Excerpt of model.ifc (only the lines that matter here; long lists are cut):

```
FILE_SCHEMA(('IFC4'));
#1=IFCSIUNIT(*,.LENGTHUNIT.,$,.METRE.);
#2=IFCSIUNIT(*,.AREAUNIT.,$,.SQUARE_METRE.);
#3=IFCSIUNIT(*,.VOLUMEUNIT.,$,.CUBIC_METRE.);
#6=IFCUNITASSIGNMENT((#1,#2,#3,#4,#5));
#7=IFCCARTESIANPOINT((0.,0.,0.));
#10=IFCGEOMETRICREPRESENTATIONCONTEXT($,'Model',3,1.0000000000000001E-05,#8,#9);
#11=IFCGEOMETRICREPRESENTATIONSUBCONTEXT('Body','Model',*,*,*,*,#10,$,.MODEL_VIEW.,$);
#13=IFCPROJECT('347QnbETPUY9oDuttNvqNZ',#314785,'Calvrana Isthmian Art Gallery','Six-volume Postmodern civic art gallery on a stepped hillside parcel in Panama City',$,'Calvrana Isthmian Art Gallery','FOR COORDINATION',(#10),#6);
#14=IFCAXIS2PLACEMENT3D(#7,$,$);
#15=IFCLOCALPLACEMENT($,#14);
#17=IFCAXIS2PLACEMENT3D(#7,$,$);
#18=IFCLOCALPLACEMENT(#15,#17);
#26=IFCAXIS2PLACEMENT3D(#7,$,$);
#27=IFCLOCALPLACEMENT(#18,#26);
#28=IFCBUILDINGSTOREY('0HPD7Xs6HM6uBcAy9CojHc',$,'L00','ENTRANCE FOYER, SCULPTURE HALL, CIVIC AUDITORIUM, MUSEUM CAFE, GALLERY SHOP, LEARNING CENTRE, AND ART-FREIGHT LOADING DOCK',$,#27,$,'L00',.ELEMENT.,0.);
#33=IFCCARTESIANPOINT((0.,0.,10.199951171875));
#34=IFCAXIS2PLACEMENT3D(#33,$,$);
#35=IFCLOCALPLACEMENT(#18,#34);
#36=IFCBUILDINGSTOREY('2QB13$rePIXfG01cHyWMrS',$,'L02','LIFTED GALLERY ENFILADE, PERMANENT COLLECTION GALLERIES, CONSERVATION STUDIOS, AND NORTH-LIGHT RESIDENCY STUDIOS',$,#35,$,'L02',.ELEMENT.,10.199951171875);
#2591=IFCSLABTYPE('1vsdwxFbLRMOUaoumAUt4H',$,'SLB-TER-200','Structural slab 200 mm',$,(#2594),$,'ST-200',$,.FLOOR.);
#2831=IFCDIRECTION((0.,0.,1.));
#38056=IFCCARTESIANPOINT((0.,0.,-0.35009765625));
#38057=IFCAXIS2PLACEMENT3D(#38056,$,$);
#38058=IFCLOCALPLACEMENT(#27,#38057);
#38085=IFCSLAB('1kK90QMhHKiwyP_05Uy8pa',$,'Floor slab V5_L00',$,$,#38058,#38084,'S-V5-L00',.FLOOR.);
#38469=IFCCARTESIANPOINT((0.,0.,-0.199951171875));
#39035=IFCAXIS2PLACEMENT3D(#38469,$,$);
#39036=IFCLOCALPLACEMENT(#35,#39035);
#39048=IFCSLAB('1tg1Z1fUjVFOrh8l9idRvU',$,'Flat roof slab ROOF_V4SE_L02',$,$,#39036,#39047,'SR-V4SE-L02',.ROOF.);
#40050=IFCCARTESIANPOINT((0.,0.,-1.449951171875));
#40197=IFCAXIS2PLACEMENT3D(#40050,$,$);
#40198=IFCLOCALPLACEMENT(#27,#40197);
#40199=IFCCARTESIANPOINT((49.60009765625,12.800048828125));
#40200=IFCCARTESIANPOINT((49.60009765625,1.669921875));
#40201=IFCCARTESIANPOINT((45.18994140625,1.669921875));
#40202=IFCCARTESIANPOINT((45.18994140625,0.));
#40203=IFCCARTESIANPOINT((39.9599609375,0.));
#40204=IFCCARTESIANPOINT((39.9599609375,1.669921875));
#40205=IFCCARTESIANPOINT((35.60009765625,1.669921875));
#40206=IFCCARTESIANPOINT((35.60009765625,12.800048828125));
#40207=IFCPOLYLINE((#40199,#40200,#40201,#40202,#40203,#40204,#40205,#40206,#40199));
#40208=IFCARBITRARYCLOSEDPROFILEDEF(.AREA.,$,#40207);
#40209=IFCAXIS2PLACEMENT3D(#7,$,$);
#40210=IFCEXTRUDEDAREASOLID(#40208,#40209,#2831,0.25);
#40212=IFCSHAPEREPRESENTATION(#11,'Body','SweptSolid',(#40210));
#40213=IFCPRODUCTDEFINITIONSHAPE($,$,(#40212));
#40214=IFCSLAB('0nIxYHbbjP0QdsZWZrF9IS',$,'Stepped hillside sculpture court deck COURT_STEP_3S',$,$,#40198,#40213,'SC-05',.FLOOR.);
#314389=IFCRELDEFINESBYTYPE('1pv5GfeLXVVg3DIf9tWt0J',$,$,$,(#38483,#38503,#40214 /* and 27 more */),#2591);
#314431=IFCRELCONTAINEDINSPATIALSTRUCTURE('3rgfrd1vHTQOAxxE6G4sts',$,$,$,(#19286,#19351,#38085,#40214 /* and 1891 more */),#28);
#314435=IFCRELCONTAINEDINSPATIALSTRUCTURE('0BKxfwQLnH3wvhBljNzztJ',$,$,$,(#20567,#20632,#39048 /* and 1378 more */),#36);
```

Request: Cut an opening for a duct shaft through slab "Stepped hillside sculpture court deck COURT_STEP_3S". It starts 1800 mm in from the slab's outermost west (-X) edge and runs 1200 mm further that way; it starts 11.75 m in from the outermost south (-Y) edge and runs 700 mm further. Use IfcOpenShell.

```python
import numpy as np
import ifcopenshell
import ifcopenshell.api.feature
import ifcopenshell.api.geometry
import ifcopenshell.api.root
import ifcopenshell.geom
import ifcopenshell.util.placement
import ifcopenshell.util.representation
import ifcopenshell.util.shape
import ifcopenshell.util.unit

model = ifcopenshell.open("model.ifc")
unit_scale = ifcopenshell.util.unit.calculate_unit_scale(model)
settings = ifcopenshell.geom.settings()


def volume(element):
    """Net volume in cubic metres, openings subtracted."""
    shape = ifcopenshell.geom.create_shape(settings, element)
    return ifcopenshell.util.shape.get_volume(shape.geometry)


slab = model.by_guid("0nIxYHbbjP0QdsZWZrF9IS")
before = volume(slab)

# Extent in the slab's own axes, in metres. The edges named are its -X and -Y sides.
slab_shape = ifcopenshell.geom.create_shape(settings, slab)
vertices = ifcopenshell.util.shape.get_vertices(slab_shape.geometry)
x_min, y_min, bottom = vertices.min(axis=0)
top = vertices[:, 2].max()

opening = ifcopenshell.api.root.create_entity(model, ifc_class="IfcOpeningElement", name="Duct shaft opening", predefined_type="OPENING")
context = ifcopenshell.util.representation.get_context(model, "Model", "Body", "MODEL_VIEW")
width, depth = 1.2, 0.7
outline = [(0.0, 0.0), (width, 0.0), (width, depth), (0.0, depth), (0.0, 0.0)]
# Overshoot both faces by 50 mm so the cut is clean.
shape = ifcopenshell.api.geometry.add_slab_representation(
    model, context=context, depth=top - bottom + 0.1, polyline=outline
)
ifcopenshell.api.geometry.assign_representation(model, product=opening, representation=shape)

matrix = ifcopenshell.util.placement.get_local_placement(slab.ObjectPlacement)
matrix[:, 3] = matrix @ np.append(np.array([x_min + 1.8, y_min + 11.75, bottom - 0.05]) / unit_scale, 1.0)
ifcopenshell.api.geometry.edit_object_placement(model, product=opening, matrix=matrix, is_si=False)
ifcopenshell.api.feature.add_feature(model, feature=opening, element=slab)

after = volume(slab)

print(f"slab volume {before:.3f} -> {after:.3f} m3")

model.write("model_edited.ifc")
```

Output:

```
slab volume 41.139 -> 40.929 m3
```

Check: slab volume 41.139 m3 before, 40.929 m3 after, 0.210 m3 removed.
